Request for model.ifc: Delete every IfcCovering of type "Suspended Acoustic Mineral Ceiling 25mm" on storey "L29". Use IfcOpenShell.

First a look at what the model holds.

```python
import ifcopenshell
import ifcopenshell.util.element

model = ifcopenshell.open("model.ifc")
print(model.schema)
storey = next(s for s in model.by_type("IfcBuildingStorey") if s.Name == "L29")
coverings = [e for e in ifcopenshell.util.element.get_decomposition(storey) if e.is_a("IfcCovering")]
seen = {}
for e in coverings:
    element_type = ifcopenshell.util.element.get_type(e)
    name = element_type.Name if element_type not in (None, e) else None
    seen[name] = seen.get(name, 0) + 1
for name, count in sorted(seen.items(), key=str):
    print(count, "x", name)
```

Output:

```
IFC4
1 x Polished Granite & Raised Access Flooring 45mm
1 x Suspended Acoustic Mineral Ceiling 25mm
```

```python
import ifcopenshell
import ifcopenshell.api.root
import ifcopenshell.util.element

model = ifcopenshell.open("model.ifc")

storey = next(s for s in model.by_type("IfcBuildingStorey") if s.Name == "L29")
coverings = [e for e in ifcopenshell.util.element.get_decomposition(storey) if e.is_a("IfcCovering")]
targets = [e for e in coverings if (t := ifcopenshell.util.element.get_type(e)) not in (None, e) and t.Name == "Suspended Acoustic Mineral Ceiling 25mm"]

for e in targets:
    ifcopenshell.api.root.remove_product(model, product=e)
print(len(targets), "removed")

model.write("model_edited.ifc")
```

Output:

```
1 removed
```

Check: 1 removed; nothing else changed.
